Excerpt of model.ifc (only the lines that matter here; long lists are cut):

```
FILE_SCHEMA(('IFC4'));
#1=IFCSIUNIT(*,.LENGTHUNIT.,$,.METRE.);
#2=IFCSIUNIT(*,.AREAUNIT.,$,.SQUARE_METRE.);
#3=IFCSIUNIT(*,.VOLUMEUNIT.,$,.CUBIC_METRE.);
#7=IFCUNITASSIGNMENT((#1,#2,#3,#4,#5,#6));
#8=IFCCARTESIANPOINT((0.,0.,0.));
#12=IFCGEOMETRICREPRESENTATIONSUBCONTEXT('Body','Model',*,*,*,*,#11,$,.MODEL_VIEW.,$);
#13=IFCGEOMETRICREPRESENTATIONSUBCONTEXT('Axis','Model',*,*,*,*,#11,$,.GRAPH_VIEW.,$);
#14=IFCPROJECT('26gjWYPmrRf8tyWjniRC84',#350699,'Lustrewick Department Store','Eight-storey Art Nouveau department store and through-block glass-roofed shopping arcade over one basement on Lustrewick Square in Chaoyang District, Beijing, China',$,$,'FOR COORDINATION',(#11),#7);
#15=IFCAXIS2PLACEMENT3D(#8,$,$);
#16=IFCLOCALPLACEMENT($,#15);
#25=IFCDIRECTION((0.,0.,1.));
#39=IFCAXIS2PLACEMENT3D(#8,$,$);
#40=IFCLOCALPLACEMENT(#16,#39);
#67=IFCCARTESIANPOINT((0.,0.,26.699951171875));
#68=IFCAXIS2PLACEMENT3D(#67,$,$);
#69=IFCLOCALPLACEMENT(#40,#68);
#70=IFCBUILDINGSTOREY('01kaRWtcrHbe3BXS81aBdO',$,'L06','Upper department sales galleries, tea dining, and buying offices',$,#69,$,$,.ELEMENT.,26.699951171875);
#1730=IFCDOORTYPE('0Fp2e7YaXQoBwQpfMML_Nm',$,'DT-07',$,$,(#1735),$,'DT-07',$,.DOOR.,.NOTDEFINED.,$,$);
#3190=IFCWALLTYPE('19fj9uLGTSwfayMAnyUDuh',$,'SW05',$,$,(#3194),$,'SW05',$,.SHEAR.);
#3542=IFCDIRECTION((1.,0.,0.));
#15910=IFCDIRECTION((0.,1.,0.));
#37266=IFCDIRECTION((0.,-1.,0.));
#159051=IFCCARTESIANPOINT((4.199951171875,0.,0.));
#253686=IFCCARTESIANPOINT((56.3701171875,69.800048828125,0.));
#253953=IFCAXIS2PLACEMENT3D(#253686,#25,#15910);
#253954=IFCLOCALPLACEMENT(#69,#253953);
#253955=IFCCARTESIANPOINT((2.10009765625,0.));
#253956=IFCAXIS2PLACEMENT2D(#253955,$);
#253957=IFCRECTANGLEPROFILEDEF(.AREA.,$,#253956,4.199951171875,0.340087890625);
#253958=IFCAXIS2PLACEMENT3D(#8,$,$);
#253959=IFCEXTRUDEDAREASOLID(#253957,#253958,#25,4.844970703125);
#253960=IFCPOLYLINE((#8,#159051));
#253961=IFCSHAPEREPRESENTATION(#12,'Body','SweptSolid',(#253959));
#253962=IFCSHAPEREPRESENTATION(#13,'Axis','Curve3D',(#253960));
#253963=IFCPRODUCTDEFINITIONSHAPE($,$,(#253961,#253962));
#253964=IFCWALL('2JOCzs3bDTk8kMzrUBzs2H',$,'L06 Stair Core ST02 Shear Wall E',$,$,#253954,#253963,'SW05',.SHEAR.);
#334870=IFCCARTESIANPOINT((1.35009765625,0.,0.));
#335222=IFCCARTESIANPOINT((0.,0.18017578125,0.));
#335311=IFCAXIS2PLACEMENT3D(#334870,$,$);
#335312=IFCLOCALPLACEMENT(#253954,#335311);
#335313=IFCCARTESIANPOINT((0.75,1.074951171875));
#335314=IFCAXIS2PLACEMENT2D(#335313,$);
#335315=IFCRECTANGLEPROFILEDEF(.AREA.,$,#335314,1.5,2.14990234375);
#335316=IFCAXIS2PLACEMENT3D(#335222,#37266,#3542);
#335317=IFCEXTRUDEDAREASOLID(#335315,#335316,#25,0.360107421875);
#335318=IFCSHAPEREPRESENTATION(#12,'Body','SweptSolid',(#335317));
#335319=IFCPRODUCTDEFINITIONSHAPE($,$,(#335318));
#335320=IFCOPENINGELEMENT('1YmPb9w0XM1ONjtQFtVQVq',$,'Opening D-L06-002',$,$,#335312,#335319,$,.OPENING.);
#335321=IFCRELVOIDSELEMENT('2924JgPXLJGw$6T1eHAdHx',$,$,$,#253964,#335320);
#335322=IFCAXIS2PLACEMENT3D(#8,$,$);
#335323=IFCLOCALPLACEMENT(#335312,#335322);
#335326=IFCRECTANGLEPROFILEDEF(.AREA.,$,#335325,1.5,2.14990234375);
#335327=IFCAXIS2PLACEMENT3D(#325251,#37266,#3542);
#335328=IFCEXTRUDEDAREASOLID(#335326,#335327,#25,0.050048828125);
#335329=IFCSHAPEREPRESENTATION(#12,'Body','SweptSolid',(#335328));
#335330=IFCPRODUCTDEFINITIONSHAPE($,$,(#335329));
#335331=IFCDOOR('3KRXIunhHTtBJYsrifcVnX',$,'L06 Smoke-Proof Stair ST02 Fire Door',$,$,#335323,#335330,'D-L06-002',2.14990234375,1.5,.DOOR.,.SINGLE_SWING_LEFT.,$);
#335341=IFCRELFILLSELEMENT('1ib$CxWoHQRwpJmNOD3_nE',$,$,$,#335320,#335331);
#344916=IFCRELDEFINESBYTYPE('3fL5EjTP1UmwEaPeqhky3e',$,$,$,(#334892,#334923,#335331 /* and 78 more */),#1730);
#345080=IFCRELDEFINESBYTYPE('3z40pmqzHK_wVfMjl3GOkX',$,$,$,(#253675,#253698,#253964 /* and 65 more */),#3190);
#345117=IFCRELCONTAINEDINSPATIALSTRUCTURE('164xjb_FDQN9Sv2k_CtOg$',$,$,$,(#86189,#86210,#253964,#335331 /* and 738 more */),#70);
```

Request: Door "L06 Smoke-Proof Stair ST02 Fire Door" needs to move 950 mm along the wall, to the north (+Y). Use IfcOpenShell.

```python
import ifcopenshell
import ifcopenshell.api.geometry
import ifcopenshell.util.placement

model = ifcopenshell.open("model.ifc")

door = model.by_guid("3KRXIunhHTtBJYsrifcVnX")
opening = door.FillsVoids[0].RelatingOpeningElement
wall = opening.VoidsElements[0].RelatingBuildingElement

wall_matrix = ifcopenshell.util.placement.get_local_placement(wall.ObjectPlacement)
shift = wall_matrix[:3, 0] * 0.95
before = ifcopenshell.util.placement.get_local_placement(door.ObjectPlacement)[:3, 3].copy()

# The door is placed relative to its opening, so it follows when the opening moves.
matrix = ifcopenshell.util.placement.get_local_placement(opening.ObjectPlacement)
matrix[:3, 3] += shift
ifcopenshell.api.geometry.edit_object_placement(
    model, product=opening, matrix=matrix, is_si=False, should_transform_children=True
)

after = ifcopenshell.util.placement.get_local_placement(door.ObjectPlacement)[:3, 3]
print("door moved by", (after - before).round(3) + 0.0)

model.write("model_edited.ifc")
```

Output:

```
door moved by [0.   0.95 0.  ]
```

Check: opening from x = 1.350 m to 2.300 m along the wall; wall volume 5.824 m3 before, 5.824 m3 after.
